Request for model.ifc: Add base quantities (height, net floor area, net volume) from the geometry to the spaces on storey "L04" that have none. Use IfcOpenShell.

First a look at what the model holds.

```python
import ifcopenshell
import ifcopenshell.util.element
import ifcopenshell.util.unit

model = ifcopenshell.open("model.ifc")
print(model.schema)
for unit_type in ("LENGTHUNIT", "AREAUNIT", "VOLUMEUNIT"):
    print(unit_type, ifcopenshell.util.unit.calculate_unit_scale(model, unit_type))
storey = next(s for s in model.by_type("IfcBuildingStorey") if s.Name == "L04")
spaces = [e for e in ifcopenshell.util.element.get_decomposition(storey) if e.is_a("IfcSpace")]
for e in sorted(spaces, key=lambda e: e.id()):
    print(e.id(), e.is_a(), e.Name, list(ifcopenshell.util.element.get_psets(e, qtos_only=True)), sep=" | ")
```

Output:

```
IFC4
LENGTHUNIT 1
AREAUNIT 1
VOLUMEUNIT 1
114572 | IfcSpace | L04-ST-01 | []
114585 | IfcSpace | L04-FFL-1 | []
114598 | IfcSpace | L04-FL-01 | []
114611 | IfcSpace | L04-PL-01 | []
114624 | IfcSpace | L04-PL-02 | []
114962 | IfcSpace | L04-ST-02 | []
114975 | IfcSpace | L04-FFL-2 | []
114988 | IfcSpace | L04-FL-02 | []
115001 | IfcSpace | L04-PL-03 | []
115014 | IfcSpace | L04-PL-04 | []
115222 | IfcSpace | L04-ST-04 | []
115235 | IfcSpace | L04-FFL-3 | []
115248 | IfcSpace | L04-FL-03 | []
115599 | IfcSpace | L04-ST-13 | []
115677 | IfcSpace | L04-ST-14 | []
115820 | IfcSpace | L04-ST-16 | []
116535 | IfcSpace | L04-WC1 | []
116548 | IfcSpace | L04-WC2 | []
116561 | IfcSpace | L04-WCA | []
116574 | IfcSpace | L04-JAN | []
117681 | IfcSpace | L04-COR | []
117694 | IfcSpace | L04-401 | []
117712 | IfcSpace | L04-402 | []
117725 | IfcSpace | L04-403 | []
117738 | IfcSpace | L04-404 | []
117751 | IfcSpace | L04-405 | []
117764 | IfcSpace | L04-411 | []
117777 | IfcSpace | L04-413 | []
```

```python
import ifcopenshell
import ifcopenshell.api.pset
import ifcopenshell.geom
import ifcopenshell.util.element
import ifcopenshell.util.shape
import ifcopenshell.util.unit

model = ifcopenshell.open("model.ifc")
unit_scale = ifcopenshell.util.unit.calculate_unit_scale(model)
area_scale = ifcopenshell.util.unit.calculate_unit_scale(model, "AREAUNIT")
volume_scale = ifcopenshell.util.unit.calculate_unit_scale(model, "VOLUMEUNIT")
settings = ifcopenshell.geom.settings()

storey = next(s for s in model.by_type("IfcBuildingStorey") if s.Name == "L04")
spaces = [e for e in ifcopenshell.util.element.get_decomposition(storey) if e.is_a("IfcSpace")]

for e in sorted(spaces, key=lambda e: e.id()):
    if ifcopenshell.util.element.get_psets(e, qtos_only=True, should_inherit=False):
        continue
    # Geometry comes back in metres, in the element's own axes.
    shape = ifcopenshell.geom.create_shape(settings, e)
    values = {
        "Height": ifcopenshell.util.shape.get_z(shape.geometry) / unit_scale,
        "NetFloorArea": ifcopenshell.util.shape.get_footprint_area(shape.geometry) / area_scale,
        "NetVolume": ifcopenshell.util.shape.get_volume(shape.geometry) / volume_scale,
    }
    qto = ifcopenshell.api.pset.add_qto(model, product=e, name="Qto_SpaceBaseQuantities")
    ifcopenshell.api.pset.edit_qto(model, qto=qto, properties=values)
    print(e.id(), {k: round(v, 3) for k, v in values.items()})

model.write("model_updated.ifc")
```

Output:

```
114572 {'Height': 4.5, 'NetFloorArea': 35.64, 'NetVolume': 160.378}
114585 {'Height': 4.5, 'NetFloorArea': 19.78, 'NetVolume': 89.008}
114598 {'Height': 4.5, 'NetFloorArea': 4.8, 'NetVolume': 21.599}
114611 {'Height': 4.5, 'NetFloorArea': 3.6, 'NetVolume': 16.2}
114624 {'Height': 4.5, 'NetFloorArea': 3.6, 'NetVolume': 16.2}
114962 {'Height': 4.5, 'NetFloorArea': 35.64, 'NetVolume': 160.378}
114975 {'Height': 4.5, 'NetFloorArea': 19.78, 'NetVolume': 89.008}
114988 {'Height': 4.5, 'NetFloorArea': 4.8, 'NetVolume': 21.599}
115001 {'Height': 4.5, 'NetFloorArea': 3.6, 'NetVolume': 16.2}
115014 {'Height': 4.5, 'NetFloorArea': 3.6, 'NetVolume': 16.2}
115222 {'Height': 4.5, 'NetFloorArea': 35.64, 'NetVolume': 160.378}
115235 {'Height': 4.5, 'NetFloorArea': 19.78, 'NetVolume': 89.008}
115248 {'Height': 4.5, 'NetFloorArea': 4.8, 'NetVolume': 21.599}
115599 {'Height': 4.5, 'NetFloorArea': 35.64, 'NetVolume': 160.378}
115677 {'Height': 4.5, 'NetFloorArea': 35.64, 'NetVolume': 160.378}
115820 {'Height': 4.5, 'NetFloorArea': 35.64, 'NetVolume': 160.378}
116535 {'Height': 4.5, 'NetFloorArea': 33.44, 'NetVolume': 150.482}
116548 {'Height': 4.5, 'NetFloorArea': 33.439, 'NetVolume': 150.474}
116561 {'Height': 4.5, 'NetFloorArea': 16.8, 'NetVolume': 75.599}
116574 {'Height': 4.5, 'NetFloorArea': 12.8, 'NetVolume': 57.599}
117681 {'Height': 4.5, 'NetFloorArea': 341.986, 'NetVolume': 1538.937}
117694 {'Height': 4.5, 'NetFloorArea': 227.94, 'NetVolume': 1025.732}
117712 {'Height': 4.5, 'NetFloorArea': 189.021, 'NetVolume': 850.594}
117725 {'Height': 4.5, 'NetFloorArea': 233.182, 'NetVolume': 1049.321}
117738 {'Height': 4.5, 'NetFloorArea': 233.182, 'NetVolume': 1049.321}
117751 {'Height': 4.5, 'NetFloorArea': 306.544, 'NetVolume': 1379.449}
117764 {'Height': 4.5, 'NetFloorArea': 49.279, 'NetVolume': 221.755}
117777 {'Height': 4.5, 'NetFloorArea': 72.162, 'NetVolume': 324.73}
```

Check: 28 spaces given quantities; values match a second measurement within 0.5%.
